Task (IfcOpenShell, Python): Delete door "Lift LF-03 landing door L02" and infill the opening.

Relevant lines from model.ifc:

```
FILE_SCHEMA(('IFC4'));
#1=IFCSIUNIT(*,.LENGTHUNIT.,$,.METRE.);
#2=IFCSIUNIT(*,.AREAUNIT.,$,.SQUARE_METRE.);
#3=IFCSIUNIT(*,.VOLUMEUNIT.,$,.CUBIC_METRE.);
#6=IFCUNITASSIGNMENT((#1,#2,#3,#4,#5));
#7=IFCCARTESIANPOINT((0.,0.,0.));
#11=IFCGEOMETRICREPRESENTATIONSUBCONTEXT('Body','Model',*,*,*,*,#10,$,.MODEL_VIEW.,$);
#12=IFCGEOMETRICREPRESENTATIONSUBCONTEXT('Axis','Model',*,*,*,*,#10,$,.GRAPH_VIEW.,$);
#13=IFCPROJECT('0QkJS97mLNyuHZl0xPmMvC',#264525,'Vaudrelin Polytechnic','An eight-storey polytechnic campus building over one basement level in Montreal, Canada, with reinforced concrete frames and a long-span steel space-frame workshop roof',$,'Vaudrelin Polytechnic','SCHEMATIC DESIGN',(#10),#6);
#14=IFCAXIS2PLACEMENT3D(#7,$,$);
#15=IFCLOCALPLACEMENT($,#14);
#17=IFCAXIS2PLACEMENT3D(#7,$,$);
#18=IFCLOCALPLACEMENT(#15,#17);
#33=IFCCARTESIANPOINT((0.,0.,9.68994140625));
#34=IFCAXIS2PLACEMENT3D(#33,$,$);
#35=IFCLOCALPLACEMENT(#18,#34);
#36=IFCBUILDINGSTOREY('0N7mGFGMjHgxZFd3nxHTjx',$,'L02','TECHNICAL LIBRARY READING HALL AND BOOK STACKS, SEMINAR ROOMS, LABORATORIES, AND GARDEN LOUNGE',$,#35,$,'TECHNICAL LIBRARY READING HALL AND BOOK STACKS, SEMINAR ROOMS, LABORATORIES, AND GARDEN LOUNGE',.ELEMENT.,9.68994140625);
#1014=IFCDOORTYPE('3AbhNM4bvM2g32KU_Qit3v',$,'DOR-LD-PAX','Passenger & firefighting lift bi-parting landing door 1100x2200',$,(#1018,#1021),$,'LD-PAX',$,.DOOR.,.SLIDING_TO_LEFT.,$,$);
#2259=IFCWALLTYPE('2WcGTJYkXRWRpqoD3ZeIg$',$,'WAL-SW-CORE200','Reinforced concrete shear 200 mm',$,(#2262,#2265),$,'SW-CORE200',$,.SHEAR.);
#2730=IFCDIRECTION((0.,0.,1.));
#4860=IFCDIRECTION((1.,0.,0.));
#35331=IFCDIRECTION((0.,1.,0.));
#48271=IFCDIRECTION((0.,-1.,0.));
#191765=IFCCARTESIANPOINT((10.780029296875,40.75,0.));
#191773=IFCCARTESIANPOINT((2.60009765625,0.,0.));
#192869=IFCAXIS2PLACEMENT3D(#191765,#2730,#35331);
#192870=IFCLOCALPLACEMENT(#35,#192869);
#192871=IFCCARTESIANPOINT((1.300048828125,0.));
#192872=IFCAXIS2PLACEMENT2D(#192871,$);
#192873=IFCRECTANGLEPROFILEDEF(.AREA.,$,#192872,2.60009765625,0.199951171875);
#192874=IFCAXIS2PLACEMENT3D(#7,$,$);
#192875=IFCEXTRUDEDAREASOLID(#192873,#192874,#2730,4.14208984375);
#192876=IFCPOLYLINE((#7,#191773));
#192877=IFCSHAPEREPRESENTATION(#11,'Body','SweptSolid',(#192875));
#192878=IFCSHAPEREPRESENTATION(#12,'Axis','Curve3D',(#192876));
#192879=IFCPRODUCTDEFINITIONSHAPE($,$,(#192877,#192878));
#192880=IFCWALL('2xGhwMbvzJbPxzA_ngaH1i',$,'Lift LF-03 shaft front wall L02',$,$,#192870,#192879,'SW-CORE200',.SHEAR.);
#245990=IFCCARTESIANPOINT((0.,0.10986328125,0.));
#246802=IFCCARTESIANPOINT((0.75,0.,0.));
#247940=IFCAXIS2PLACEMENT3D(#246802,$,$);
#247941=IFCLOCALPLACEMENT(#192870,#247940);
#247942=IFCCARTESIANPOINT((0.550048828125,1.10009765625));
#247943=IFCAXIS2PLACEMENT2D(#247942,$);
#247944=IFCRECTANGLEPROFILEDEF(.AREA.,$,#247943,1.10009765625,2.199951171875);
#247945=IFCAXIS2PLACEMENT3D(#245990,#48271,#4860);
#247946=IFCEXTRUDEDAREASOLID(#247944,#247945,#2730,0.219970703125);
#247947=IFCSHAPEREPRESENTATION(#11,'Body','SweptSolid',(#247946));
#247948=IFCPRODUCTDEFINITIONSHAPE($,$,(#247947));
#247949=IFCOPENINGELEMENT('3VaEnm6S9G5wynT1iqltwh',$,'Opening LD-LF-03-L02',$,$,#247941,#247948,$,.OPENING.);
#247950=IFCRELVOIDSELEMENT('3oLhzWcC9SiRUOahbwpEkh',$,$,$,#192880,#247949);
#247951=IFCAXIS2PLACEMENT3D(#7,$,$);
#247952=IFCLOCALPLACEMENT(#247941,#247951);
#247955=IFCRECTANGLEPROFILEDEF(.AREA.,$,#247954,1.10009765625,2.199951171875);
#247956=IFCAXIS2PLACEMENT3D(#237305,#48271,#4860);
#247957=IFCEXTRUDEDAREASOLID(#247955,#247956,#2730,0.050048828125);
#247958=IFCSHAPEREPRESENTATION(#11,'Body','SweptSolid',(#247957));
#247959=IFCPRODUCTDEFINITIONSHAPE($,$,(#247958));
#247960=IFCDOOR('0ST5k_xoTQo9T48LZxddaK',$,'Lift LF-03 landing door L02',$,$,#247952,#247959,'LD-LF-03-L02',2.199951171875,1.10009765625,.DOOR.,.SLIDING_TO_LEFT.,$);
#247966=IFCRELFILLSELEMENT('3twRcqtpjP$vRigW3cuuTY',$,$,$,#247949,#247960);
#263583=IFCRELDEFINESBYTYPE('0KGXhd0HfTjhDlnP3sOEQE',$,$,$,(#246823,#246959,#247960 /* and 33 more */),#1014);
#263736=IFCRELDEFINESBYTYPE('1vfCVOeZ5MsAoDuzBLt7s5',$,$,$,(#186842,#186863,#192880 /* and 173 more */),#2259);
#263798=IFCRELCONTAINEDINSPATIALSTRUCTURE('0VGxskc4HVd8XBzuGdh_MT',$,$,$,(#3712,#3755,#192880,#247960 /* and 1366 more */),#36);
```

```python
import ifcopenshell
import ifcopenshell.api.feature
import ifcopenshell.api.root
import ifcopenshell.geom
import ifcopenshell.util.shape

model = ifcopenshell.open("model.ifc")
settings = ifcopenshell.geom.settings()


def volume(element):
    """Net volume in cubic metres, openings subtracted."""
    shape = ifcopenshell.geom.create_shape(settings, element)
    return ifcopenshell.util.shape.get_volume(shape.geometry)


door = model.by_guid("0ST5k_xoTQo9T48LZxddaK")
opening = door.FillsVoids[0].RelatingOpeningElement
wall = opening.VoidsElements[0].RelatingBuildingElement
before = volume(wall)

ifcopenshell.api.root.remove_product(model, product=door)
ifcopenshell.api.feature.remove_feature(model, feature=opening)

after = volume(wall)

print(f"wall volume {before:.3f} -> {after:.3f} m3")

model.write("model_rev.ifc")
```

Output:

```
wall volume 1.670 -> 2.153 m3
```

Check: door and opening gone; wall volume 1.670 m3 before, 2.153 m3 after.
